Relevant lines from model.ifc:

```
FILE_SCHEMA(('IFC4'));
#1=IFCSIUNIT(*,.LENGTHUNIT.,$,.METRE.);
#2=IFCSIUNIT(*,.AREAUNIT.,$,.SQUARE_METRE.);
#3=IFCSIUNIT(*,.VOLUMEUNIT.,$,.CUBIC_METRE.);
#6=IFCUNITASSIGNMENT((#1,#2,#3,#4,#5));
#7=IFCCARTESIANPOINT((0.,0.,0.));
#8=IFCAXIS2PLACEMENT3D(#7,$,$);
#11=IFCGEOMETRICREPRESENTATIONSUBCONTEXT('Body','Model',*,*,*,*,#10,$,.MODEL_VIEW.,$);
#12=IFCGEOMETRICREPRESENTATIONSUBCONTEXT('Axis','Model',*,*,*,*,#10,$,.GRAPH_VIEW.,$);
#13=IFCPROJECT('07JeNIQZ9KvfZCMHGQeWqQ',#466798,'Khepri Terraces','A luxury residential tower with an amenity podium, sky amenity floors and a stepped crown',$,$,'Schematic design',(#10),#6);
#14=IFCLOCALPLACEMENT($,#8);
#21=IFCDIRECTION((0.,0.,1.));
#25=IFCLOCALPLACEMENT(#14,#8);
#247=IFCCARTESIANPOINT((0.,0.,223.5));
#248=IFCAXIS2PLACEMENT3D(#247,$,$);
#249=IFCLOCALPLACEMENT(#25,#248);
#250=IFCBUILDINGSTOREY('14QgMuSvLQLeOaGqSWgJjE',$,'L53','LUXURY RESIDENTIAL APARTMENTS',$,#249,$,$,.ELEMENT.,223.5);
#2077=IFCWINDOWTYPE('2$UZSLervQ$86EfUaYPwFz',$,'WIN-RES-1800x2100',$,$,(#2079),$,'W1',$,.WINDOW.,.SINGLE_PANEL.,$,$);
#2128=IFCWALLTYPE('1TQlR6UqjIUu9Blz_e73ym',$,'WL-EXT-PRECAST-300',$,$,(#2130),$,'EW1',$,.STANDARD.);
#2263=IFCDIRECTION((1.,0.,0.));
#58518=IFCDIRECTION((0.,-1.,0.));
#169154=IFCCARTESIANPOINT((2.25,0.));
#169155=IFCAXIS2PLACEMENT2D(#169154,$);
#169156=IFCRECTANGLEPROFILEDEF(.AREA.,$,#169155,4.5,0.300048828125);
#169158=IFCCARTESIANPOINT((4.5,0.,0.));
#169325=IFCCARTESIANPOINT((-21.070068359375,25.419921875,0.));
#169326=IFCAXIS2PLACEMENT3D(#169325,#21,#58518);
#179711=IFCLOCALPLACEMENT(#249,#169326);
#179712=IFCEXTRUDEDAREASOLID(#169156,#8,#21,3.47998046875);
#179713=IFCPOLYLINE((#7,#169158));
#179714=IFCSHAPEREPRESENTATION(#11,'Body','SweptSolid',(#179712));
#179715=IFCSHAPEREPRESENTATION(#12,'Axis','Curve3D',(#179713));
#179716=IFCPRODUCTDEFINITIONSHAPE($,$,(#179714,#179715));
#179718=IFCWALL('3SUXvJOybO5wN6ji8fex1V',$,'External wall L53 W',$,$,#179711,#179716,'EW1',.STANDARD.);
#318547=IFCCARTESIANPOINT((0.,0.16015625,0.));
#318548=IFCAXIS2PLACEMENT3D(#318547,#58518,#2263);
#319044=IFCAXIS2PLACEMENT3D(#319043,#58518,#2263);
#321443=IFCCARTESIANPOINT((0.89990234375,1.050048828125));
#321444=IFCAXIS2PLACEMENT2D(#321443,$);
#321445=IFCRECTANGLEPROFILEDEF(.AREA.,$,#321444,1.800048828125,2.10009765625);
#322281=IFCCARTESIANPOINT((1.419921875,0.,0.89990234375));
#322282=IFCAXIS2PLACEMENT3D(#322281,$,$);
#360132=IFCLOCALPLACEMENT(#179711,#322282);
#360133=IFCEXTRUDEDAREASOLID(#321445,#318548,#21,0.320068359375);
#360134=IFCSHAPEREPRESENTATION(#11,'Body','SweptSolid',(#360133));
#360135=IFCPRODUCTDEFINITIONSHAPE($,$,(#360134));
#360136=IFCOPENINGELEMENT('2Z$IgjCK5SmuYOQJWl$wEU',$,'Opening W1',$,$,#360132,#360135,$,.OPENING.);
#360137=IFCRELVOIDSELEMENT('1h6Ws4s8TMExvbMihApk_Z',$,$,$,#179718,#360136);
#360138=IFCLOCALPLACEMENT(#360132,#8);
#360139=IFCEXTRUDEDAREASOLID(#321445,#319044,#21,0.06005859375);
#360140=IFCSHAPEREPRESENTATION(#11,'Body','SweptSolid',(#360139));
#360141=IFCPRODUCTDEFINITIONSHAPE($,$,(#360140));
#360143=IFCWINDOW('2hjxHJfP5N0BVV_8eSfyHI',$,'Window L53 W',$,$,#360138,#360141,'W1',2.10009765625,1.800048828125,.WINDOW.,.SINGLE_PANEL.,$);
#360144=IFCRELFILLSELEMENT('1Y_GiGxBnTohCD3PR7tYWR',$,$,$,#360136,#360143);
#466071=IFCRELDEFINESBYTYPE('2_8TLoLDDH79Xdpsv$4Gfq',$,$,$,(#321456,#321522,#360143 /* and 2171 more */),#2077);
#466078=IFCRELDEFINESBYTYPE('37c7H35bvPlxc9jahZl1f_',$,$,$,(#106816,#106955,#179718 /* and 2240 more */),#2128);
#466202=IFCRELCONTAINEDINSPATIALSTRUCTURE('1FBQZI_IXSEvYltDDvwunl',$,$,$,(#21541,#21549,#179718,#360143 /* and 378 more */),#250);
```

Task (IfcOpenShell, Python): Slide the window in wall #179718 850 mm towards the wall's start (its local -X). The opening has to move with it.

```python
import ifcopenshell
import ifcopenshell.api.geometry
import ifcopenshell.util.placement
import ifcopenshell.util.unit

model = ifcopenshell.open("model.ifc")
unit_scale = ifcopenshell.util.unit.calculate_unit_scale(model)

window = model.by_id(360143)
opening = window.FillsVoids[0].RelatingOpeningElement
wall = opening.VoidsElements[0].RelatingBuildingElement

wall_matrix = ifcopenshell.util.placement.get_local_placement(wall.ObjectPlacement)
shift = wall_matrix[:3, 0] * -0.85 / unit_scale
before = ifcopenshell.util.placement.get_local_placement(window.ObjectPlacement)[:3, 3].copy()

# The window is placed relative to its opening, so it follows when the opening moves.
matrix = ifcopenshell.util.placement.get_local_placement(opening.ObjectPlacement)
matrix[:3, 3] += shift
ifcopenshell.api.geometry.edit_object_placement(
    model, product=opening, matrix=matrix, is_si=False, should_transform_children=True
)

after = ifcopenshell.util.placement.get_local_placement(window.ObjectPlacement)[:3, 3]
print("window moved by", (after - before).round(3) + 0.0)

model.write("model_edited.ifc")
```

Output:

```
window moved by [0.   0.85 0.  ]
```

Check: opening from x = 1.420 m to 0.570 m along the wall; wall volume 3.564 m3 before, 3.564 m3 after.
